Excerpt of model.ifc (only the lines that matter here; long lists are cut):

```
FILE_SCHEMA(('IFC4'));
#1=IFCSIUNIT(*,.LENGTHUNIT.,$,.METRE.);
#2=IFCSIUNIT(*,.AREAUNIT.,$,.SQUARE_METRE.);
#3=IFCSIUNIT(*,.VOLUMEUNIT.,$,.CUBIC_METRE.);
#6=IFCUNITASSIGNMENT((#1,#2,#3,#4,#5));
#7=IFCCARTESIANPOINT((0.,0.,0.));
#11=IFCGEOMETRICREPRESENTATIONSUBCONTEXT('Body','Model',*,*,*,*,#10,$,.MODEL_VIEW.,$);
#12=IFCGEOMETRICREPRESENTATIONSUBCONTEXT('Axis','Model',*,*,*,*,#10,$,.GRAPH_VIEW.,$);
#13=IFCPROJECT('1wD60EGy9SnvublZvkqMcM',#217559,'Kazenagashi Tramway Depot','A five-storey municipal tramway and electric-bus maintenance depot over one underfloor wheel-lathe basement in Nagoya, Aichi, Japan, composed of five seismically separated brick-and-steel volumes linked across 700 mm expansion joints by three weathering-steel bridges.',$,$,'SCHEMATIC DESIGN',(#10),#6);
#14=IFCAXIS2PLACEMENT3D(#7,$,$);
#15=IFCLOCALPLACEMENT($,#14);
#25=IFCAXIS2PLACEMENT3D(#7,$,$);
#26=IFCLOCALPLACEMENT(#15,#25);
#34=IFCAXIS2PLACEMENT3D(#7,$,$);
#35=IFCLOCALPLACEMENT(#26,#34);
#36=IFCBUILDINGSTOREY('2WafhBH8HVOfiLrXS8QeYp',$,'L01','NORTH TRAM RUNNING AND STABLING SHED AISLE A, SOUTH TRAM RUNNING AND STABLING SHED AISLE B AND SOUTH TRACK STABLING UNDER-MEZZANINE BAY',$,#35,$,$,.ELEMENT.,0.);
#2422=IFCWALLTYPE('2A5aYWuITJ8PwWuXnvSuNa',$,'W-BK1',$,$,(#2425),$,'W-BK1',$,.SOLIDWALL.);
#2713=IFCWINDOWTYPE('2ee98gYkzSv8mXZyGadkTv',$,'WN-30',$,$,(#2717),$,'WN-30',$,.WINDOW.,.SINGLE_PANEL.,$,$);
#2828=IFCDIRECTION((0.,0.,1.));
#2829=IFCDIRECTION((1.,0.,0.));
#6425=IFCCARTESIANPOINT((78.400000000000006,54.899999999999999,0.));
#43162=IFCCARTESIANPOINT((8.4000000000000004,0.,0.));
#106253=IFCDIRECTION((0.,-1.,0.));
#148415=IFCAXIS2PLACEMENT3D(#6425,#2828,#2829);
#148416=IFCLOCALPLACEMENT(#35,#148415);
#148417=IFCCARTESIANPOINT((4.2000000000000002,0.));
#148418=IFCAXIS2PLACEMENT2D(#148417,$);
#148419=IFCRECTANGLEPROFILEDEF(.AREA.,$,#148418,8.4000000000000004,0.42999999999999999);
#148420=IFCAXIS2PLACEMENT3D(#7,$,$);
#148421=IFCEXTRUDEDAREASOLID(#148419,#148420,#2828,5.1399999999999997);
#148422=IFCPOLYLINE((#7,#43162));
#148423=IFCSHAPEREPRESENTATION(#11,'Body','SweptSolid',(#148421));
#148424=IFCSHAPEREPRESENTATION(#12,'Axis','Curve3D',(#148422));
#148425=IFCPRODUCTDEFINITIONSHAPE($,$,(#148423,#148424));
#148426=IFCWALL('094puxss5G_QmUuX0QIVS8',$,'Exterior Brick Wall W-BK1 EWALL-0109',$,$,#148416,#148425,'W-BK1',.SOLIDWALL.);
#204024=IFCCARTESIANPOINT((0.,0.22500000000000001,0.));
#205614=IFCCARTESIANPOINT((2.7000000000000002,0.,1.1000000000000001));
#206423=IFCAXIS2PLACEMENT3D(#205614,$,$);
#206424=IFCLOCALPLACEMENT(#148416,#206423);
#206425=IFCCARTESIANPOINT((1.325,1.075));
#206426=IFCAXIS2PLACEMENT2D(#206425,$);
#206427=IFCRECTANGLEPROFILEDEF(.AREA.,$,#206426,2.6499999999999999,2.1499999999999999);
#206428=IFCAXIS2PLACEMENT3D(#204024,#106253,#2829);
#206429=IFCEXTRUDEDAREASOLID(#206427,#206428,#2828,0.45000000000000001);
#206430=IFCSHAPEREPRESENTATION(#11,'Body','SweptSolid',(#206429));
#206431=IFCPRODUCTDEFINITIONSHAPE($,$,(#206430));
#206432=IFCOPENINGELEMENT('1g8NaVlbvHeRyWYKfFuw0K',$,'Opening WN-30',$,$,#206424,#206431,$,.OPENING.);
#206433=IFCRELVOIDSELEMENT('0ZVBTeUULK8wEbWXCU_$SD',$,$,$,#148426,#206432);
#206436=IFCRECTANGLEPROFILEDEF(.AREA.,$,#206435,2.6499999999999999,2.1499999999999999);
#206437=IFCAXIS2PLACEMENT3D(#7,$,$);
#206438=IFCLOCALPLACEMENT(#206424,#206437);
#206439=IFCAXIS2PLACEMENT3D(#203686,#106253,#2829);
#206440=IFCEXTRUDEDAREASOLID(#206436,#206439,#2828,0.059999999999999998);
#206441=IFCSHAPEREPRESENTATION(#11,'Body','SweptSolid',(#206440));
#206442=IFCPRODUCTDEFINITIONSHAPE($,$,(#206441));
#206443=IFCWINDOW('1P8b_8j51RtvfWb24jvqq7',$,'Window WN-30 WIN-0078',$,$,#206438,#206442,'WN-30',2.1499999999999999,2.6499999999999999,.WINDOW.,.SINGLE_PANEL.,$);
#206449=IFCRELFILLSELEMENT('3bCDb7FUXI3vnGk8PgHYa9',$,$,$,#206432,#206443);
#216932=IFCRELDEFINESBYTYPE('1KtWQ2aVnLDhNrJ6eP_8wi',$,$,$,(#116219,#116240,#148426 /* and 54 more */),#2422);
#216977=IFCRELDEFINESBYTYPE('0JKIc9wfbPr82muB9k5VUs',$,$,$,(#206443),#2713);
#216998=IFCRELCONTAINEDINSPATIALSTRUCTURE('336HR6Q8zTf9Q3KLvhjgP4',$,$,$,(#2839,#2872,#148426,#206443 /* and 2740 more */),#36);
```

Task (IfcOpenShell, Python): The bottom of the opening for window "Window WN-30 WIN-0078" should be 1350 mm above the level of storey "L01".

```python
import numpy as np
import ifcopenshell
import ifcopenshell.api.geometry
import ifcopenshell.geom
import ifcopenshell.util.element
import ifcopenshell.util.placement
import ifcopenshell.util.shape
import ifcopenshell.util.unit

model = ifcopenshell.open("model.ifc")
unit_scale = ifcopenshell.util.unit.calculate_unit_scale(model)

window = model.by_guid("1P8b_8j51RtvfWb24jvqq7")
opening = window.FillsVoids[0].RelatingOpeningElement
storey = ifcopenshell.util.element.get_container(window, ifc_class="IfcBuildingStorey")
level = ifcopenshell.util.placement.get_local_placement(storey.ObjectPlacement)[2, 3]

# The opening's origin need not be at the sill, so measure its lowest point.
shape = ifcopenshell.geom.create_shape(ifcopenshell.geom.settings(), opening)
bottom = ifcopenshell.util.shape.get_shape_bottom_elevation(shape, shape.geometry) / unit_scale
dz = level + 1.35 - bottom

shift = np.array([0.0, 0.0, dz])
# The window is placed relative to its opening, so it follows when the opening moves.
matrix = ifcopenshell.util.placement.get_local_placement(opening.ObjectPlacement)
matrix[:3, 3] += shift
ifcopenshell.api.geometry.edit_object_placement(
    model, product=opening, matrix=matrix, is_si=False, should_transform_children=True
)

print(f"moved by {dz * unit_scale:+.3f} m")

model.write("model_rev.ifc")
```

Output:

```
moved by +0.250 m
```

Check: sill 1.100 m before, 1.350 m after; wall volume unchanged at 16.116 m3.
